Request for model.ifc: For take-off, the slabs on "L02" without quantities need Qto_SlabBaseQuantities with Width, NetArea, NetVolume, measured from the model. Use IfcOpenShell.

First a look at what the model holds.

```python
import ifcopenshell
import ifcopenshell.util.element
import ifcopenshell.util.unit

model = ifcopenshell.open("model.ifc")
print(model.schema)
for unit_type in ("LENGTHUNIT", "AREAUNIT", "VOLUMEUNIT"):
    print(unit_type, ifcopenshell.util.unit.calculate_unit_scale(model, unit_type))
storey = next(s for s in model.by_type("IfcBuildingStorey") if s.Name == "L02")
slabs = [e for e in ifcopenshell.util.element.get_decomposition(storey) if e.is_a("IfcSlab")]
for e in sorted(slabs, key=lambda e: e.id()):
    print(e.id(), e.is_a(), e.Name, list(ifcopenshell.util.element.get_psets(e, qtos_only=True)), sep=" | ")
```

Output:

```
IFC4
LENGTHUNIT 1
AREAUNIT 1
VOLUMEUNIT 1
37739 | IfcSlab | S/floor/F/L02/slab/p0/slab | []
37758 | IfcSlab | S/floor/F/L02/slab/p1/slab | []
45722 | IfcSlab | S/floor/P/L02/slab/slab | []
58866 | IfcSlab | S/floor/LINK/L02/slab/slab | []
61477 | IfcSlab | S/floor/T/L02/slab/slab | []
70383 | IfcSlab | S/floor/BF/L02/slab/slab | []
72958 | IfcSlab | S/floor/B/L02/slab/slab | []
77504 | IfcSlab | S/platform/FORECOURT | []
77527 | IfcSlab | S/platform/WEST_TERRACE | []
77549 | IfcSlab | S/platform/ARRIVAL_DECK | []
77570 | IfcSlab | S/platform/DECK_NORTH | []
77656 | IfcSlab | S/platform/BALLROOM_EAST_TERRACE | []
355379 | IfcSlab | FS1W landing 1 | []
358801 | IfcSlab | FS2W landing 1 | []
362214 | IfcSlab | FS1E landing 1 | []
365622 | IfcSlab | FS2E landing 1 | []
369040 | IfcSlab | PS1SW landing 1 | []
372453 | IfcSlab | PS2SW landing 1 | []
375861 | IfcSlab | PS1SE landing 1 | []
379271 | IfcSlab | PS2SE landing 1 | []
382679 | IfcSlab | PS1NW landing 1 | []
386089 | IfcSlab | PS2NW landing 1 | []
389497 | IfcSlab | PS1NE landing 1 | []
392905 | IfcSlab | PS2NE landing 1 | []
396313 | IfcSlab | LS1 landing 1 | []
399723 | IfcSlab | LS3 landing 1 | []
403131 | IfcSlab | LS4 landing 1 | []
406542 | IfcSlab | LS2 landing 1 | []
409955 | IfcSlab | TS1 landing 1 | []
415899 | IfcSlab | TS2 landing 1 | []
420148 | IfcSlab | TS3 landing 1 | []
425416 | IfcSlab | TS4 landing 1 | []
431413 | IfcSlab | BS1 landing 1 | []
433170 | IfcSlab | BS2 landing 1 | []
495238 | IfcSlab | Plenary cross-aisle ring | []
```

```python
import ifcopenshell
import ifcopenshell.api.pset
import ifcopenshell.geom
import ifcopenshell.util.element
import ifcopenshell.util.shape
import ifcopenshell.util.unit

model = ifcopenshell.open("model.ifc")
unit_scale = ifcopenshell.util.unit.calculate_unit_scale(model)
area_scale = ifcopenshell.util.unit.calculate_unit_scale(model, "AREAUNIT")
volume_scale = ifcopenshell.util.unit.calculate_unit_scale(model, "VOLUMEUNIT")
settings = ifcopenshell.geom.settings()

storey = next(s for s in model.by_type("IfcBuildingStorey") if s.Name == "L02")
slabs = [e for e in ifcopenshell.util.element.get_decomposition(storey) if e.is_a("IfcSlab")]

for e in sorted(slabs, key=lambda e: e.id()):
    if ifcopenshell.util.element.get_psets(e, qtos_only=True, should_inherit=False):
        continue
    # Geometry comes back in metres, in the element's own axes.
    shape = ifcopenshell.geom.create_shape(settings, e)
    values = {
        "Width": ifcopenshell.util.shape.get_z(shape.geometry) / unit_scale,
        "NetArea": ifcopenshell.util.shape.get_footprint_area(shape.geometry) / area_scale,
        "NetVolume": ifcopenshell.util.shape.get_volume(shape.geometry) / volume_scale,
    }
    qto = ifcopenshell.api.pset.add_qto(model, product=e, name="Qto_SlabBaseQuantities")
    ifcopenshell.api.pset.edit_qto(model, qto=qto, properties=values)
    print(e.id(), {k: round(v, 3) for k, v in values.items()})

model.write("model_updated.ifc")
```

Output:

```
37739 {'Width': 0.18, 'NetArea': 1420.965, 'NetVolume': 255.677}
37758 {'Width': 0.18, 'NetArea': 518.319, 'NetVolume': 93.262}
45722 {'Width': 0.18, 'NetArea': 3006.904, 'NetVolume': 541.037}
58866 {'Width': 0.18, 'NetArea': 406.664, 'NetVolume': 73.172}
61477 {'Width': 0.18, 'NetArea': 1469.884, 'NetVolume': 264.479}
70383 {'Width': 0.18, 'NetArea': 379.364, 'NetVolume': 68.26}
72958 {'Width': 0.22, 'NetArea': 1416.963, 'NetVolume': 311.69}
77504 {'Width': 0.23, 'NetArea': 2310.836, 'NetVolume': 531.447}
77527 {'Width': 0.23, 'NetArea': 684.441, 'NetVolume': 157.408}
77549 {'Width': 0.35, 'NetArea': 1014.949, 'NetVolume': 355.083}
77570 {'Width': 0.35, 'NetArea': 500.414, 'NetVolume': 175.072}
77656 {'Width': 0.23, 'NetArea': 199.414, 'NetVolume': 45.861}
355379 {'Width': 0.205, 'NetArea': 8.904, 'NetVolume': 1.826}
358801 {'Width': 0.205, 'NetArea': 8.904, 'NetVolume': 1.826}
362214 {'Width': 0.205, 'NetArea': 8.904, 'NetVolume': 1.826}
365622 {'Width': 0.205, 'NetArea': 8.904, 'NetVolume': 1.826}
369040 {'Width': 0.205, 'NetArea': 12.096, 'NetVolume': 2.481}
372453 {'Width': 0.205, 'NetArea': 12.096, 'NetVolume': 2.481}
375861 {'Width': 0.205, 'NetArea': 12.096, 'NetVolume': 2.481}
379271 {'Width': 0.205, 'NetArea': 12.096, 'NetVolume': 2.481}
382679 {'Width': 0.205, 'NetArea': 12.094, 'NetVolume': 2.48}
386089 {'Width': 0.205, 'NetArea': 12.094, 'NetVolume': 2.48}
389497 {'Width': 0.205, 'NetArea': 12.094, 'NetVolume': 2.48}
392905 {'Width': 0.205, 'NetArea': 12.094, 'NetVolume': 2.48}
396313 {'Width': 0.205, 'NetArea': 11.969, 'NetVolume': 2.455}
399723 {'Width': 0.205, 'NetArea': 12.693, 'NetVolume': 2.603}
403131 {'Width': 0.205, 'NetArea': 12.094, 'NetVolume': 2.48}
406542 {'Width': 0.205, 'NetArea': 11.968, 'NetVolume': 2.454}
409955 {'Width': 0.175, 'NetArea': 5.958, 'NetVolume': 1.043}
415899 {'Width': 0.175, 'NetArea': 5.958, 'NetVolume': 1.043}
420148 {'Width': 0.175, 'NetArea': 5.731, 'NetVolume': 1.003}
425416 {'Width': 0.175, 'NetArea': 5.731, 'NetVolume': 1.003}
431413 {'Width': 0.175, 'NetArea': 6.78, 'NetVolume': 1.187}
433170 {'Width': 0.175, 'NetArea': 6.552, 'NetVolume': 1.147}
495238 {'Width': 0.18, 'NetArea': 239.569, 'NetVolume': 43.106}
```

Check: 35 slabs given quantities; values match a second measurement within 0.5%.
